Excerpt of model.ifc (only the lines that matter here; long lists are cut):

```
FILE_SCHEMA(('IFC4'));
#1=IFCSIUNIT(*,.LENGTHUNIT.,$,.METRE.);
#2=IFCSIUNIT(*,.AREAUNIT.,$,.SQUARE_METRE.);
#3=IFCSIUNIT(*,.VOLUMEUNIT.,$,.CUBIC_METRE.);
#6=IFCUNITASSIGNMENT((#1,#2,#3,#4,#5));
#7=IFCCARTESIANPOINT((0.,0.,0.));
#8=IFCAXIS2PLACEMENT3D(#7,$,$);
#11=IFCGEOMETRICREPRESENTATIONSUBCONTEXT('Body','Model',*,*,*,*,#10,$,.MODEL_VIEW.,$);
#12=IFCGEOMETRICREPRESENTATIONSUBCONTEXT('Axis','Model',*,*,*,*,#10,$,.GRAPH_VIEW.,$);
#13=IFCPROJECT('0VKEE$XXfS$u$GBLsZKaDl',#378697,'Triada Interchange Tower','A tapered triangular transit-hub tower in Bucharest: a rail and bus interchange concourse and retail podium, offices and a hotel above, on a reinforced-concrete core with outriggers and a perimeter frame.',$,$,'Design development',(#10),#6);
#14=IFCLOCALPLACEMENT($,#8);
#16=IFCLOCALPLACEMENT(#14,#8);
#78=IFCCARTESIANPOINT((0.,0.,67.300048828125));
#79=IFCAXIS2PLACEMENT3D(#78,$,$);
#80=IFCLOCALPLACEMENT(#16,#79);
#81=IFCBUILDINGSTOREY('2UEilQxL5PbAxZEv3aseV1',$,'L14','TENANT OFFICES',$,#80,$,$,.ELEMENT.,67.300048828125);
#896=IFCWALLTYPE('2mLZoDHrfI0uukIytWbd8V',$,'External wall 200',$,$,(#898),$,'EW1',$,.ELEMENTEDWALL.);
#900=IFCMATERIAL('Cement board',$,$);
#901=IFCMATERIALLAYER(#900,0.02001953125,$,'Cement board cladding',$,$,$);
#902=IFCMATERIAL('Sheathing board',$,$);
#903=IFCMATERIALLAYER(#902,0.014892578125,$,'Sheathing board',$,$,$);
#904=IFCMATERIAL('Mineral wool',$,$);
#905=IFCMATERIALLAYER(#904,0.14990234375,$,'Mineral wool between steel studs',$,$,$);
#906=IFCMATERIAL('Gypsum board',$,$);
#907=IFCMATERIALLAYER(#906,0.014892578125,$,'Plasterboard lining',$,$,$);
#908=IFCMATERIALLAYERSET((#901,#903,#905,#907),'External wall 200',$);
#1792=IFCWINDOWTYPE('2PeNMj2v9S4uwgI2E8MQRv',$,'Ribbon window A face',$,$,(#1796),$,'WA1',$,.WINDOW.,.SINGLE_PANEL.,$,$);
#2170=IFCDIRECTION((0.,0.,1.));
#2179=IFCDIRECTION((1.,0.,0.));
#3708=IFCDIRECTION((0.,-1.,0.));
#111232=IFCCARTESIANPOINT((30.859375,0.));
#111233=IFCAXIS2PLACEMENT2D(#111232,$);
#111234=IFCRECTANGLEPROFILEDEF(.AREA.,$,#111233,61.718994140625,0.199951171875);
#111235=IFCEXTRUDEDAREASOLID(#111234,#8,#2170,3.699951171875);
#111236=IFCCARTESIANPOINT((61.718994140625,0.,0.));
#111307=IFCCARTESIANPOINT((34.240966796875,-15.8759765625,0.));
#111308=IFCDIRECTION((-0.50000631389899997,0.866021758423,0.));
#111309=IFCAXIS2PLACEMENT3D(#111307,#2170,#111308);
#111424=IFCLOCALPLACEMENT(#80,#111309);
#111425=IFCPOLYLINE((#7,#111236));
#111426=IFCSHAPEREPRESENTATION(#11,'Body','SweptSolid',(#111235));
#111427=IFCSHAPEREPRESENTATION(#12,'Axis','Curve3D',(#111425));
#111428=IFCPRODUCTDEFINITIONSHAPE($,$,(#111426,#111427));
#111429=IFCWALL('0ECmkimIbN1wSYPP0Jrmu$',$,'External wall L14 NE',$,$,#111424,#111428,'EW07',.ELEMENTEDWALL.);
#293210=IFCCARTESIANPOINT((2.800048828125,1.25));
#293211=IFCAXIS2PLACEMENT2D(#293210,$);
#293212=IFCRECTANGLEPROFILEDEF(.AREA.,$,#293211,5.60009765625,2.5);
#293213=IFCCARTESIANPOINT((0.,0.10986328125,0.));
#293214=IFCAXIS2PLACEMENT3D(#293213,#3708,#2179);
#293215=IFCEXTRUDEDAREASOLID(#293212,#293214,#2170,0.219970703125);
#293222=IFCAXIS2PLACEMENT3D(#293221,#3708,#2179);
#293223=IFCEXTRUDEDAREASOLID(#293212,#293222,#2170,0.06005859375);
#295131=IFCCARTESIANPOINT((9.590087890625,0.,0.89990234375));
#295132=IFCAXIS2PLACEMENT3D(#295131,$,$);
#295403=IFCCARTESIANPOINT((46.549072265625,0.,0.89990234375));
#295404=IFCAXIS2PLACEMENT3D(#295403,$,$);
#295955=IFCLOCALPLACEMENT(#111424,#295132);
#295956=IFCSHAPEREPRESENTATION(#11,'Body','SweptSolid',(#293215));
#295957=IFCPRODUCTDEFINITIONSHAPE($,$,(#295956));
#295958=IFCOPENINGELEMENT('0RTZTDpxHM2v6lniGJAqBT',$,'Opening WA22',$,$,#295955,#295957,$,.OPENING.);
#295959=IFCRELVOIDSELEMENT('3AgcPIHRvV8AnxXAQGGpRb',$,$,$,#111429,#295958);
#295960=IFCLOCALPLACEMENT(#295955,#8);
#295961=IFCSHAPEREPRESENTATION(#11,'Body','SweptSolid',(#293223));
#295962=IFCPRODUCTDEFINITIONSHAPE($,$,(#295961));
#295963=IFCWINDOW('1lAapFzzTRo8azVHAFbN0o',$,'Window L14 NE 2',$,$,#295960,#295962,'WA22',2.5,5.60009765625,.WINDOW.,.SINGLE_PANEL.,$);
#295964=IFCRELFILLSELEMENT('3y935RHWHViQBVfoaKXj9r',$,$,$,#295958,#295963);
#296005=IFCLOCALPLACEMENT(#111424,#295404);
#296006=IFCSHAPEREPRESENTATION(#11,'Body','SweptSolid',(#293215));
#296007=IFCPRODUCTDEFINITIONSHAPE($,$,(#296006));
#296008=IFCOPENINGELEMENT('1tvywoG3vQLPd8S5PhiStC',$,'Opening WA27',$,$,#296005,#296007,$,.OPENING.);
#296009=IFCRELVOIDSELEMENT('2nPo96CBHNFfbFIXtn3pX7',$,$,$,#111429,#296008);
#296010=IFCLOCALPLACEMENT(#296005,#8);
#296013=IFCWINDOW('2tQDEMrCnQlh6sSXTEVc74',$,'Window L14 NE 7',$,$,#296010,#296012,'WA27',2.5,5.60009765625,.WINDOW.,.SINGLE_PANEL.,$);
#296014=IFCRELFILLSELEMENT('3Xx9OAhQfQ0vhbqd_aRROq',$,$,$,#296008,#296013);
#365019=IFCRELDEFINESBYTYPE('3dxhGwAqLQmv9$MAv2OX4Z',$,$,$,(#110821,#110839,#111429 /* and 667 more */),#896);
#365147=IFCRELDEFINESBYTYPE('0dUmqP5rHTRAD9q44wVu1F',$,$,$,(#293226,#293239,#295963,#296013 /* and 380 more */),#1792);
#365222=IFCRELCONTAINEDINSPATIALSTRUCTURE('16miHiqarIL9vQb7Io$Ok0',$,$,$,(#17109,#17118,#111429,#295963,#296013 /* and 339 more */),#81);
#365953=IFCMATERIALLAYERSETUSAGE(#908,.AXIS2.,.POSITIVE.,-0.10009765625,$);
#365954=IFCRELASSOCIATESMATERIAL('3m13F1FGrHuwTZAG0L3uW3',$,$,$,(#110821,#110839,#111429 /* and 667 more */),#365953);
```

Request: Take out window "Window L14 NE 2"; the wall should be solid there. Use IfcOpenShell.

```python
import ifcopenshell
import ifcopenshell.api.feature
import ifcopenshell.api.root
import ifcopenshell.geom
import ifcopenshell.util.shape

model = ifcopenshell.open("model.ifc")
settings = ifcopenshell.geom.settings()


def volume(element):
    """Net volume in cubic metres, openings subtracted."""
    shape = ifcopenshell.geom.create_shape(settings, element)
    return ifcopenshell.util.shape.get_volume(shape.geometry)


window = model.by_id(295963)
opening = window.FillsVoids[0].RelatingOpeningElement
wall = opening.VoidsElements[0].RelatingBuildingElement
before = volume(wall)

ifcopenshell.api.root.remove_product(model, product=window)
ifcopenshell.api.feature.remove_feature(model, feature=opening)

after = volume(wall)

print(f"wall volume {before:.3f} -> {after:.3f} m3")

model.write("model-out.ifc")
```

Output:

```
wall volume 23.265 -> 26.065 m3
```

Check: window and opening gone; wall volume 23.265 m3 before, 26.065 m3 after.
